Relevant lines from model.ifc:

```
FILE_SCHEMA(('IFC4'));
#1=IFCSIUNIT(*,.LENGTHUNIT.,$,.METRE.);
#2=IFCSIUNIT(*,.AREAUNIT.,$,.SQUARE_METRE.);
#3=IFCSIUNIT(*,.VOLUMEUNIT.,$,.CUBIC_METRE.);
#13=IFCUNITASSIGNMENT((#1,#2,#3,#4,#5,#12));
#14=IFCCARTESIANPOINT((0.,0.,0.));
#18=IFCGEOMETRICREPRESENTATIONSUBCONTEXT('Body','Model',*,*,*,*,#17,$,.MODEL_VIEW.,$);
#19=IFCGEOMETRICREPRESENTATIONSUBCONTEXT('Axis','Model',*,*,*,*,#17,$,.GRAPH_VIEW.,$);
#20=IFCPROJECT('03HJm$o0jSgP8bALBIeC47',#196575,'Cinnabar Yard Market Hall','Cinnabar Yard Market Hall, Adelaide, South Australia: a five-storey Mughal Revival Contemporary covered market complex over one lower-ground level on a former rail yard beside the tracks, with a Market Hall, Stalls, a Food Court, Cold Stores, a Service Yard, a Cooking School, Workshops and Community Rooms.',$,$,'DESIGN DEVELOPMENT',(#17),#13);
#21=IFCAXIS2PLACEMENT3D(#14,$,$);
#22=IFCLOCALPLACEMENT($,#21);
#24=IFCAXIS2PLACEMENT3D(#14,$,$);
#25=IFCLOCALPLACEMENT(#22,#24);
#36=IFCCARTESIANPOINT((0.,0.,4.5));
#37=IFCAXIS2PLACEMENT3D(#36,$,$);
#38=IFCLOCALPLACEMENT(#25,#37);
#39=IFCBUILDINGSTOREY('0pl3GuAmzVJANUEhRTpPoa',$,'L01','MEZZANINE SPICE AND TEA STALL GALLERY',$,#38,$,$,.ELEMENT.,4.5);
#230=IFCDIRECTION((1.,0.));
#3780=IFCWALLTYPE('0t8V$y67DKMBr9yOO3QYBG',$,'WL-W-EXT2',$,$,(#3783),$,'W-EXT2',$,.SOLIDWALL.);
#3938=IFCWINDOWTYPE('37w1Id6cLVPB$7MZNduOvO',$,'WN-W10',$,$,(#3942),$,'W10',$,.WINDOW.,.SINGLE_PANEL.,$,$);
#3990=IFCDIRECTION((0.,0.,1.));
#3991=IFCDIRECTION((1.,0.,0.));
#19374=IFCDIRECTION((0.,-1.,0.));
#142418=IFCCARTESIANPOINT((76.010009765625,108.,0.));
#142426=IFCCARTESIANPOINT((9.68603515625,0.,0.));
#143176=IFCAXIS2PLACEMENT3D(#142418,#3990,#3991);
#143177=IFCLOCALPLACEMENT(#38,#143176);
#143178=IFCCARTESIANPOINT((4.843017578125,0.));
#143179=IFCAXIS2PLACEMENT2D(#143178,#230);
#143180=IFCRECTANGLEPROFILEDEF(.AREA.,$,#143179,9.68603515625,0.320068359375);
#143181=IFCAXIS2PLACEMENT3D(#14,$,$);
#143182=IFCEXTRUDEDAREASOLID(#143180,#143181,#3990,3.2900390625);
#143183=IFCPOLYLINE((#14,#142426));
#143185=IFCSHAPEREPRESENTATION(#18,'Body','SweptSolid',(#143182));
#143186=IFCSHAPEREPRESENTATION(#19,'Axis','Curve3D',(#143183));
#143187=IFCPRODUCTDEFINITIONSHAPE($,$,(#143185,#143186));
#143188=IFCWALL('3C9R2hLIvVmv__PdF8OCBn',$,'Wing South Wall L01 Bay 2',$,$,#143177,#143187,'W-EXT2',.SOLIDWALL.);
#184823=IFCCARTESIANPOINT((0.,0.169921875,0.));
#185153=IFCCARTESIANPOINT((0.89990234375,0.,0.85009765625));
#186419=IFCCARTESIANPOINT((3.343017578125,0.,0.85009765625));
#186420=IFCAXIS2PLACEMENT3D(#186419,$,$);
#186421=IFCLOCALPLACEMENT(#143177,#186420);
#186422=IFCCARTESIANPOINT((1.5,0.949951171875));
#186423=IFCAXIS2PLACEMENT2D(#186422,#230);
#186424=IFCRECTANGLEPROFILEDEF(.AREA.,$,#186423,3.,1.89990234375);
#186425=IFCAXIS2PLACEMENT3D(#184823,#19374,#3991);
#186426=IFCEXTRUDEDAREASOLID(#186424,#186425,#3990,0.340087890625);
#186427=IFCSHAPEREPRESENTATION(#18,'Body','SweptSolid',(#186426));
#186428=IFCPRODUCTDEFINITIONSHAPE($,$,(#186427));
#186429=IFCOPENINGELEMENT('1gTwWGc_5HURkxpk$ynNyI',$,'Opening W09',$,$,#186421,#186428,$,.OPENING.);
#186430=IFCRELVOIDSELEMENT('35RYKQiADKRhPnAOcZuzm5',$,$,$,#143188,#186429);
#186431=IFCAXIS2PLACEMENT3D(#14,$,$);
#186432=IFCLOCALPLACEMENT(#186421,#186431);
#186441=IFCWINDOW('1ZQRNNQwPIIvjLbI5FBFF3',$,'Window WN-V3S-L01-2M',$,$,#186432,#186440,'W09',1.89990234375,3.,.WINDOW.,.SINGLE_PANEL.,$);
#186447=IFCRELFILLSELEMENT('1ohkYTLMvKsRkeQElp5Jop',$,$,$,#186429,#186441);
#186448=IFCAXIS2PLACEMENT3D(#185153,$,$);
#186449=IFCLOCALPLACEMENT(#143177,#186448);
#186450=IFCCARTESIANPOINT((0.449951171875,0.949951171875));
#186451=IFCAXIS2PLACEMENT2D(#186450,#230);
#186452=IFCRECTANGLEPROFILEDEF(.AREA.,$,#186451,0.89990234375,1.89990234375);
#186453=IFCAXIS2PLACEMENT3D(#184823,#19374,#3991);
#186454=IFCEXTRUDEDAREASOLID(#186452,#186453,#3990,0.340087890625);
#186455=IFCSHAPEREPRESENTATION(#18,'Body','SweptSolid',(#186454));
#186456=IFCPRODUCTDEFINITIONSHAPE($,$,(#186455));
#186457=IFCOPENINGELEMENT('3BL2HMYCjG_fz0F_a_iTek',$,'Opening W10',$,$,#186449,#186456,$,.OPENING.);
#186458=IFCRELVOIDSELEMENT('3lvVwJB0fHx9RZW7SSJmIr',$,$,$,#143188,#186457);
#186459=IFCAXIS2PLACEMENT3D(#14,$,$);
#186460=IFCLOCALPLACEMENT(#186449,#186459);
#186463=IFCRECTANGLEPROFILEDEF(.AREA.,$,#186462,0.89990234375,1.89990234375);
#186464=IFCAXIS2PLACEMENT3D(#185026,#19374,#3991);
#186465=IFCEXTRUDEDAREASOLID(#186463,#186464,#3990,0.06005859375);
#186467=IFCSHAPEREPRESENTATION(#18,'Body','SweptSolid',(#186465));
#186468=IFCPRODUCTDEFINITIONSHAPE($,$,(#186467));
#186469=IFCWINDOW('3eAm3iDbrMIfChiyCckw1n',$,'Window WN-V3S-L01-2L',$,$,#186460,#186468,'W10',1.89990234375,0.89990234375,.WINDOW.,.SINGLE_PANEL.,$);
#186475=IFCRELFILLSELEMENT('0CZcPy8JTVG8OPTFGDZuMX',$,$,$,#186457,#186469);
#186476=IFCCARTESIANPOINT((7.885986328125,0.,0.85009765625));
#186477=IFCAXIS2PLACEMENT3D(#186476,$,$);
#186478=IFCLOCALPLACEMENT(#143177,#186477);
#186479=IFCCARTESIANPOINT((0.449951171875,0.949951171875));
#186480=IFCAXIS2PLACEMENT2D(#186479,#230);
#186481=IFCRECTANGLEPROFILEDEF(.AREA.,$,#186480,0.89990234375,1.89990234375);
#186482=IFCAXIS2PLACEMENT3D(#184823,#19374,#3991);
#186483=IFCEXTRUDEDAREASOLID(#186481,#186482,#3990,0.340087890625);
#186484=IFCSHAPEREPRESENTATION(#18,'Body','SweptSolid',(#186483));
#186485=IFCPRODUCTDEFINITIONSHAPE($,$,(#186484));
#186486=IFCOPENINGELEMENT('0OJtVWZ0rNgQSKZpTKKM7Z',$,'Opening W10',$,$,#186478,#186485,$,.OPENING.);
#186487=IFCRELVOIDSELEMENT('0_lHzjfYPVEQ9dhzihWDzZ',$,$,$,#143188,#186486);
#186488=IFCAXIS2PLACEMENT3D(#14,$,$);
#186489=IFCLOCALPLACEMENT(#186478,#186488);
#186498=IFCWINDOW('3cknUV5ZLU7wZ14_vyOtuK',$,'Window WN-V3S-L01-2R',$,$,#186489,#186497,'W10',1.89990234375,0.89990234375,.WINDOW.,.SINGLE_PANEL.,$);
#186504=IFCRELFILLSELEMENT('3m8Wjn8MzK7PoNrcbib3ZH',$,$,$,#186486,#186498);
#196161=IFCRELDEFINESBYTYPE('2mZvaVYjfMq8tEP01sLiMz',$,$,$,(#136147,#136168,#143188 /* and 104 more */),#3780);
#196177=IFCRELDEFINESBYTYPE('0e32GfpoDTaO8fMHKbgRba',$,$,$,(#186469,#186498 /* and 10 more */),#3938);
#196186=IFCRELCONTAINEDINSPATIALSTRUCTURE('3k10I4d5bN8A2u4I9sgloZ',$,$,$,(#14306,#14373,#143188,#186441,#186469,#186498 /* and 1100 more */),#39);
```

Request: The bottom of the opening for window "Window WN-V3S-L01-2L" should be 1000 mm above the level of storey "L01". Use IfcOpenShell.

```python
import numpy as np
import ifcopenshell
import ifcopenshell.api.geometry
import ifcopenshell.geom
import ifcopenshell.util.element
import ifcopenshell.util.placement
import ifcopenshell.util.shape
import ifcopenshell.util.unit

model = ifcopenshell.open("model.ifc")
unit_scale = ifcopenshell.util.unit.calculate_unit_scale(model)

window = model.by_guid("3eAm3iDbrMIfChiyCckw1n")
opening = window.FillsVoids[0].RelatingOpeningElement
storey = ifcopenshell.util.element.get_container(window, ifc_class="IfcBuildingStorey")
level = ifcopenshell.util.placement.get_local_placement(storey.ObjectPlacement)[2, 3]

# The opening's origin need not be at the sill, so measure its lowest point.
shape = ifcopenshell.geom.create_shape(ifcopenshell.geom.settings(), opening)
bottom = ifcopenshell.util.shape.get_shape_bottom_elevation(shape, shape.geometry) / unit_scale
dz = level + 1.0 - bottom

shift = np.array([0.0, 0.0, dz])
# The window is placed relative to its opening, so it follows when the opening moves.
matrix = ifcopenshell.util.placement.get_local_placement(opening.ObjectPlacement)
matrix[:3, 3] += shift
ifcopenshell.api.geometry.edit_object_placement(
    model, product=opening, matrix=matrix, is_si=False, should_transform_children=True
)

print(f"moved by {dz * unit_scale:+.3f} m")

model.write("model-out.ifc")
```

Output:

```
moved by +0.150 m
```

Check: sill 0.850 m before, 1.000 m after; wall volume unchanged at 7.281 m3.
